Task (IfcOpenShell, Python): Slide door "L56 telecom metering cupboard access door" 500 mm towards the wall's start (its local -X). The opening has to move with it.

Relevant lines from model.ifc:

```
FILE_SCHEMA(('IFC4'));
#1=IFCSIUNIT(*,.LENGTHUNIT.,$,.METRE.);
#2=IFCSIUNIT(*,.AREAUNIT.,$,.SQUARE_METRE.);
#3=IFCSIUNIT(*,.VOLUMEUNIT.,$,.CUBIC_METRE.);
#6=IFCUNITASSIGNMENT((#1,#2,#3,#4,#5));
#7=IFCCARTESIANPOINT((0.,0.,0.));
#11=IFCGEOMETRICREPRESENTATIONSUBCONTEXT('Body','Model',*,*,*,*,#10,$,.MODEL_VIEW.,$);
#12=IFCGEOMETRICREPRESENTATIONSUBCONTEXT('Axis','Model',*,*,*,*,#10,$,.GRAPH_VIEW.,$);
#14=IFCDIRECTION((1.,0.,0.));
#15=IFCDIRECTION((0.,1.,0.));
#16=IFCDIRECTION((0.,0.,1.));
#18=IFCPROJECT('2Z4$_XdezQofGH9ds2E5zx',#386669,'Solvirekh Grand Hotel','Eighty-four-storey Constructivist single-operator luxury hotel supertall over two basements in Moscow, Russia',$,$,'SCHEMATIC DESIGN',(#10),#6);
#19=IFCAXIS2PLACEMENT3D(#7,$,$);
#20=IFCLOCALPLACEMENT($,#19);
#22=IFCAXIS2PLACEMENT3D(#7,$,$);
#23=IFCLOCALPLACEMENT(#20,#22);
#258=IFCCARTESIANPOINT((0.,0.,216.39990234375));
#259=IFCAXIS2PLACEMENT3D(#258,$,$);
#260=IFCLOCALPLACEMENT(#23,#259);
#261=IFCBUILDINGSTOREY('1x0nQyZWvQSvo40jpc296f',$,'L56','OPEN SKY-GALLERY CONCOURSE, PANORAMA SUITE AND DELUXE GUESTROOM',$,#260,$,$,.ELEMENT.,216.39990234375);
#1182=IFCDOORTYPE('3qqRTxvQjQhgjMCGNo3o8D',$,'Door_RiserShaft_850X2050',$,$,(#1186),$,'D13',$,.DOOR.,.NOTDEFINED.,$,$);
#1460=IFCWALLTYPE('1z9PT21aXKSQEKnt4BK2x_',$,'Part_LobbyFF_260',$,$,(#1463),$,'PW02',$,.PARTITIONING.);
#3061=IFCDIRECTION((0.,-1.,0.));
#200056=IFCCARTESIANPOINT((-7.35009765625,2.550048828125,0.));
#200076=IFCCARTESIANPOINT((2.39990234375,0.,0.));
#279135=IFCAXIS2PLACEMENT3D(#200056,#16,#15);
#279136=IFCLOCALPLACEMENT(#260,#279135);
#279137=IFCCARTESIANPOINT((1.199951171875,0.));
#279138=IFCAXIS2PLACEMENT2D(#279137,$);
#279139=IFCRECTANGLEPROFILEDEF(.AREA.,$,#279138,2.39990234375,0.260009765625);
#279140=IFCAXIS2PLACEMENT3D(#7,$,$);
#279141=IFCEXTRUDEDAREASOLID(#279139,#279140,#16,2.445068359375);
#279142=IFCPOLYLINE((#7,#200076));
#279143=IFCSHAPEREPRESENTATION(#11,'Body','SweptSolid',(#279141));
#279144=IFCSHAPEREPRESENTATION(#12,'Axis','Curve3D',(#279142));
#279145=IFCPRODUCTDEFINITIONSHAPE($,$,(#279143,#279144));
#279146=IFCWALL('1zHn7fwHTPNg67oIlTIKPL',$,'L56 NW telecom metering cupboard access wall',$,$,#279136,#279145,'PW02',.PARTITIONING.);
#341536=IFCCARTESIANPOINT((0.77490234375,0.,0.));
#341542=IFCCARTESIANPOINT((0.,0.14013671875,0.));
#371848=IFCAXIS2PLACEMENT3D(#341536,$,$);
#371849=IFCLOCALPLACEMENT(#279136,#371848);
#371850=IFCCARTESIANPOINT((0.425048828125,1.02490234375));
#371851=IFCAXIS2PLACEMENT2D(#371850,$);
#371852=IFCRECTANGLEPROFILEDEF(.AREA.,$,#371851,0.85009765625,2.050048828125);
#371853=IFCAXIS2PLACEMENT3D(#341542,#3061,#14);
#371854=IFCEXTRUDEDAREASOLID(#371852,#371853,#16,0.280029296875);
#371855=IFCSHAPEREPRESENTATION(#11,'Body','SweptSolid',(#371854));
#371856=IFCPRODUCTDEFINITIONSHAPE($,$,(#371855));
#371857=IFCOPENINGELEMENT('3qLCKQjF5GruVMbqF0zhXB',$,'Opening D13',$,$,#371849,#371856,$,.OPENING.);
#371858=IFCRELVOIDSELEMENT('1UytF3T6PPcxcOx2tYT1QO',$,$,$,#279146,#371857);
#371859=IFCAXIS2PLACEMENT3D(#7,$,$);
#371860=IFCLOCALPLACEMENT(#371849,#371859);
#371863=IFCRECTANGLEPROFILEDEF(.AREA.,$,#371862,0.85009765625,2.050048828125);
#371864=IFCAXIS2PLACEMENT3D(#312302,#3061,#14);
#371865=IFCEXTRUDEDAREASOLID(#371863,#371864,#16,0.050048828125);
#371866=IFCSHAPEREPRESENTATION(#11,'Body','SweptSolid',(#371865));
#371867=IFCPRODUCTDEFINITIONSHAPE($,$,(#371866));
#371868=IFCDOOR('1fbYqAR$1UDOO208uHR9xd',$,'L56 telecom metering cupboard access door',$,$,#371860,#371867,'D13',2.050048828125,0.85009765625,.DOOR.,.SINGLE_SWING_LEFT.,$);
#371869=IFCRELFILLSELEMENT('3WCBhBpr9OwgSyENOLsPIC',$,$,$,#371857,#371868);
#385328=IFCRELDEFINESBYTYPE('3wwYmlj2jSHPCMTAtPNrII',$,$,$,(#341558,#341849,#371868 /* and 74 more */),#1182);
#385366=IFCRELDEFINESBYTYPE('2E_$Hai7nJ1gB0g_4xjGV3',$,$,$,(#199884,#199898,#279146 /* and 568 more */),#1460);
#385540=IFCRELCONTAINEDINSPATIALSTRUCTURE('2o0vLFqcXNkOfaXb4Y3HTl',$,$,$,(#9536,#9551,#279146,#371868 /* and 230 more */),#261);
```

```python
import ifcopenshell
import ifcopenshell.api.geometry
import ifcopenshell.util.placement

model = ifcopenshell.open("model.ifc")

door = model.by_guid("1fbYqAR$1UDOO208uHR9xd")
opening = door.FillsVoids[0].RelatingOpeningElement
wall = opening.VoidsElements[0].RelatingBuildingElement

wall_matrix = ifcopenshell.util.placement.get_local_placement(wall.ObjectPlacement)
shift = wall_matrix[:3, 0] * -0.5
before = ifcopenshell.util.placement.get_local_placement(door.ObjectPlacement)[:3, 3].copy()

# The door is placed relative to its opening, so it follows when the opening moves.
matrix = ifcopenshell.util.placement.get_local_placement(opening.ObjectPlacement)
matrix[:3, 3] += shift
ifcopenshell.api.geometry.edit_object_placement(
    model, product=opening, matrix=matrix, is_si=False, should_transform_children=True
)

after = ifcopenshell.util.placement.get_local_placement(door.ObjectPlacement)[:3, 3]
print("door moved by", (after - before).round(3) + 0.0)

model.write("model_v2.ifc")
```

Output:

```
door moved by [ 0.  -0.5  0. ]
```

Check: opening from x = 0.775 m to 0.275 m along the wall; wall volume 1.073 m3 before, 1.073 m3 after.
